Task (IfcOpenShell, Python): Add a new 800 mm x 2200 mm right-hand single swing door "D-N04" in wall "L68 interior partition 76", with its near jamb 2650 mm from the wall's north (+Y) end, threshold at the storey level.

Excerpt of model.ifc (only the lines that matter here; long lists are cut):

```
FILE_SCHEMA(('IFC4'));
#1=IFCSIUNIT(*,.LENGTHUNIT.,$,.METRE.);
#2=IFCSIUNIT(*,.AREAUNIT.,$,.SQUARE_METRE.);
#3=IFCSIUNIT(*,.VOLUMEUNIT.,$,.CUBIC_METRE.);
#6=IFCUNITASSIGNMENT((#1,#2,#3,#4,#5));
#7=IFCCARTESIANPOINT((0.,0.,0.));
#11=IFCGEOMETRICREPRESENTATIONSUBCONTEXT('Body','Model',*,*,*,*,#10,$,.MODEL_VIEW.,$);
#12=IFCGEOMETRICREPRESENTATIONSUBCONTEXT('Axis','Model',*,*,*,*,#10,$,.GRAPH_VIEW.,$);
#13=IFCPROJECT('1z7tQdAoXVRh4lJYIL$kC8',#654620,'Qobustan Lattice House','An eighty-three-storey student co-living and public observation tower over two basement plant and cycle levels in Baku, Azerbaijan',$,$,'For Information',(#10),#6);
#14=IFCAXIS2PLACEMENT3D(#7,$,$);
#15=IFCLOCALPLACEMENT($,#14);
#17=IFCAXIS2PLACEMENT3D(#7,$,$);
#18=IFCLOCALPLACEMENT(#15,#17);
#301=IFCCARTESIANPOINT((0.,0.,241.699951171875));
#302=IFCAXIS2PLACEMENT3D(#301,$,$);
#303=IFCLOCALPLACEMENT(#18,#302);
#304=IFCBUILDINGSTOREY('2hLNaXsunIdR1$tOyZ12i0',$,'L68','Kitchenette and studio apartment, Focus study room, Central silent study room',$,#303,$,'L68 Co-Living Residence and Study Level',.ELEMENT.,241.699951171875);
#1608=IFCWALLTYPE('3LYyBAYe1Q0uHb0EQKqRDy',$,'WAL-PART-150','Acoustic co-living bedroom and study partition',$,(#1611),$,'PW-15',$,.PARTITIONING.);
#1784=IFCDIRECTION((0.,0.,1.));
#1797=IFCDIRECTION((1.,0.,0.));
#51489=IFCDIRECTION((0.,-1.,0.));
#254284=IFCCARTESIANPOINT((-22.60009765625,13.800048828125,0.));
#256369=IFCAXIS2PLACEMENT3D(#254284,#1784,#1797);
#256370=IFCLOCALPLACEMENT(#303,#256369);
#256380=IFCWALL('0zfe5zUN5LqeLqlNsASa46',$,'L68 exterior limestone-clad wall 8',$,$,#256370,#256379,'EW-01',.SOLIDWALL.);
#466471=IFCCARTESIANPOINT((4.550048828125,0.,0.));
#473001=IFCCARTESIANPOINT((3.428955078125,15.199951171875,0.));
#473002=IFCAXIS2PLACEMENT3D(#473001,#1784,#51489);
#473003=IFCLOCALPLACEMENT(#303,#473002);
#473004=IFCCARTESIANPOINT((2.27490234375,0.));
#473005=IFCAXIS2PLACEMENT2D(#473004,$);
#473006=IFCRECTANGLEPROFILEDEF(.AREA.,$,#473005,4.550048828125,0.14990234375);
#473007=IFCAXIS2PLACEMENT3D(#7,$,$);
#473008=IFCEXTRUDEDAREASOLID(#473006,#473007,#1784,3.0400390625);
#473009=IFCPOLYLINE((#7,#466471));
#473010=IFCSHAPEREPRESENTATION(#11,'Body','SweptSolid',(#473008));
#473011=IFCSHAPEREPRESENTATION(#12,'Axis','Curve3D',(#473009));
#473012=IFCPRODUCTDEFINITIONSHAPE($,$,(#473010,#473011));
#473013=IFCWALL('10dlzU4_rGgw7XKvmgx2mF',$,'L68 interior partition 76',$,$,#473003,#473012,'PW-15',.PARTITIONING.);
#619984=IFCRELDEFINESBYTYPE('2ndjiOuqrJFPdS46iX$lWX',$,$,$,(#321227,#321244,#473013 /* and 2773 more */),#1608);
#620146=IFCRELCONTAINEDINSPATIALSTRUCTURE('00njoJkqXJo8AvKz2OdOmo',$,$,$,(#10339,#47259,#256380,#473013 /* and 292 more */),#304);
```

```python
import numpy as np
import ifcopenshell
import ifcopenshell.api.feature
import ifcopenshell.api.geometry
import ifcopenshell.api.root
import ifcopenshell.api.spatial
import ifcopenshell.geom
import ifcopenshell.util.element
import ifcopenshell.util.placement
import ifcopenshell.util.representation
import ifcopenshell.util.shape
import ifcopenshell.util.unit

model = ifcopenshell.open("model.ifc")
unit_scale = ifcopenshell.util.unit.calculate_unit_scale(model)
settings = ifcopenshell.geom.settings()


def volume(element):
    """Net volume in cubic metres, openings subtracted."""
    shape = ifcopenshell.geom.create_shape(settings, element)
    return ifcopenshell.util.shape.get_volume(shape.geometry)


wall = model.by_guid("10dlzU4_rGgw7XKvmgx2mF")
storey = ifcopenshell.util.element.get_container(wall, ifc_class="IfcBuildingStorey")
context = ifcopenshell.util.representation.get_context(model, "Model", "Body", "MODEL_VIEW")
before = volume(wall)

width, height, from_end, sill = 0.8, 2.2, 2.65, 0.0  # metres

# The wall runs along its own X axis, and the end named is its -X end.
wall_shape = ifcopenshell.geom.create_shape(settings, wall)
x, y, z = ifcopenshell.util.shape.get_vertices(wall_shape.geometry).T
start = x.min() + from_end
face, thickness = float(y.min()), float(y.max() - y.min())
wall_matrix = ifcopenshell.util.placement.get_local_placement(wall.ObjectPlacement)
level = ifcopenshell.util.placement.get_local_placement(storey.ObjectPlacement)[2, 3]


def in_wall(x, y):
    """Placement at x, y metres in the wall's axes, at sill height."""
    matrix = wall_matrix.copy()
    matrix[:, 3] = wall_matrix @ np.array([x / unit_scale, y / unit_scale, 0.0, 1.0])
    matrix[2, 3] = level + sill / unit_scale
    return matrix


# Opening: a box that overshoots both wall faces by 50 mm.
opening = ifcopenshell.api.root.create_entity(model, ifc_class="IfcOpeningElement", predefined_type="OPENING")
box = ifcopenshell.api.geometry.add_wall_representation(
    model, context=context, length=width, height=height, thickness=thickness + 0.1
)
ifcopenshell.api.geometry.assign_representation(model, product=opening, representation=box)
ifcopenshell.api.geometry.edit_object_placement(model, product=opening, matrix=in_wall(start, face - 0.05), is_si=False)
ifcopenshell.api.feature.add_feature(model, feature=opening, element=wall)

door = ifcopenshell.api.root.create_entity(model, ifc_class="IfcDoor", name="D-N04", predefined_type="DOOR")
door.OverallWidth, door.OverallHeight = width / unit_scale, height / unit_scale
door.OperationType = "SINGLE_SWING_RIGHT"
body = ifcopenshell.api.geometry.add_door_representation(
    model,
    context=context,
    overall_width=door.OverallWidth,
    overall_height=door.OverallHeight,
    operation_type="SINGLE_SWING_RIGHT",
    lining_properties={"LiningDepth": thickness / unit_scale, "ThresholdDepth": thickness / unit_scale},
)
ifcopenshell.api.geometry.assign_representation(model, product=door, representation=body)
ifcopenshell.api.spatial.assign_container(model, products=[door], relating_structure=storey)
ifcopenshell.api.feature.add_filling(model, opening=opening, element=door)

# The lining spans the wall, so the door starts at the wall face.
ifcopenshell.api.geometry.edit_object_placement(model, product=door, matrix=in_wall(start, face), is_si=False)

after = volume(wall)

print(f"wall volume {before:.3f} -> {after:.3f} m3")

model.write("model_updated.ifc")
```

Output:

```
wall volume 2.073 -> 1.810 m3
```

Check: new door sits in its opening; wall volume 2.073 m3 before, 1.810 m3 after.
